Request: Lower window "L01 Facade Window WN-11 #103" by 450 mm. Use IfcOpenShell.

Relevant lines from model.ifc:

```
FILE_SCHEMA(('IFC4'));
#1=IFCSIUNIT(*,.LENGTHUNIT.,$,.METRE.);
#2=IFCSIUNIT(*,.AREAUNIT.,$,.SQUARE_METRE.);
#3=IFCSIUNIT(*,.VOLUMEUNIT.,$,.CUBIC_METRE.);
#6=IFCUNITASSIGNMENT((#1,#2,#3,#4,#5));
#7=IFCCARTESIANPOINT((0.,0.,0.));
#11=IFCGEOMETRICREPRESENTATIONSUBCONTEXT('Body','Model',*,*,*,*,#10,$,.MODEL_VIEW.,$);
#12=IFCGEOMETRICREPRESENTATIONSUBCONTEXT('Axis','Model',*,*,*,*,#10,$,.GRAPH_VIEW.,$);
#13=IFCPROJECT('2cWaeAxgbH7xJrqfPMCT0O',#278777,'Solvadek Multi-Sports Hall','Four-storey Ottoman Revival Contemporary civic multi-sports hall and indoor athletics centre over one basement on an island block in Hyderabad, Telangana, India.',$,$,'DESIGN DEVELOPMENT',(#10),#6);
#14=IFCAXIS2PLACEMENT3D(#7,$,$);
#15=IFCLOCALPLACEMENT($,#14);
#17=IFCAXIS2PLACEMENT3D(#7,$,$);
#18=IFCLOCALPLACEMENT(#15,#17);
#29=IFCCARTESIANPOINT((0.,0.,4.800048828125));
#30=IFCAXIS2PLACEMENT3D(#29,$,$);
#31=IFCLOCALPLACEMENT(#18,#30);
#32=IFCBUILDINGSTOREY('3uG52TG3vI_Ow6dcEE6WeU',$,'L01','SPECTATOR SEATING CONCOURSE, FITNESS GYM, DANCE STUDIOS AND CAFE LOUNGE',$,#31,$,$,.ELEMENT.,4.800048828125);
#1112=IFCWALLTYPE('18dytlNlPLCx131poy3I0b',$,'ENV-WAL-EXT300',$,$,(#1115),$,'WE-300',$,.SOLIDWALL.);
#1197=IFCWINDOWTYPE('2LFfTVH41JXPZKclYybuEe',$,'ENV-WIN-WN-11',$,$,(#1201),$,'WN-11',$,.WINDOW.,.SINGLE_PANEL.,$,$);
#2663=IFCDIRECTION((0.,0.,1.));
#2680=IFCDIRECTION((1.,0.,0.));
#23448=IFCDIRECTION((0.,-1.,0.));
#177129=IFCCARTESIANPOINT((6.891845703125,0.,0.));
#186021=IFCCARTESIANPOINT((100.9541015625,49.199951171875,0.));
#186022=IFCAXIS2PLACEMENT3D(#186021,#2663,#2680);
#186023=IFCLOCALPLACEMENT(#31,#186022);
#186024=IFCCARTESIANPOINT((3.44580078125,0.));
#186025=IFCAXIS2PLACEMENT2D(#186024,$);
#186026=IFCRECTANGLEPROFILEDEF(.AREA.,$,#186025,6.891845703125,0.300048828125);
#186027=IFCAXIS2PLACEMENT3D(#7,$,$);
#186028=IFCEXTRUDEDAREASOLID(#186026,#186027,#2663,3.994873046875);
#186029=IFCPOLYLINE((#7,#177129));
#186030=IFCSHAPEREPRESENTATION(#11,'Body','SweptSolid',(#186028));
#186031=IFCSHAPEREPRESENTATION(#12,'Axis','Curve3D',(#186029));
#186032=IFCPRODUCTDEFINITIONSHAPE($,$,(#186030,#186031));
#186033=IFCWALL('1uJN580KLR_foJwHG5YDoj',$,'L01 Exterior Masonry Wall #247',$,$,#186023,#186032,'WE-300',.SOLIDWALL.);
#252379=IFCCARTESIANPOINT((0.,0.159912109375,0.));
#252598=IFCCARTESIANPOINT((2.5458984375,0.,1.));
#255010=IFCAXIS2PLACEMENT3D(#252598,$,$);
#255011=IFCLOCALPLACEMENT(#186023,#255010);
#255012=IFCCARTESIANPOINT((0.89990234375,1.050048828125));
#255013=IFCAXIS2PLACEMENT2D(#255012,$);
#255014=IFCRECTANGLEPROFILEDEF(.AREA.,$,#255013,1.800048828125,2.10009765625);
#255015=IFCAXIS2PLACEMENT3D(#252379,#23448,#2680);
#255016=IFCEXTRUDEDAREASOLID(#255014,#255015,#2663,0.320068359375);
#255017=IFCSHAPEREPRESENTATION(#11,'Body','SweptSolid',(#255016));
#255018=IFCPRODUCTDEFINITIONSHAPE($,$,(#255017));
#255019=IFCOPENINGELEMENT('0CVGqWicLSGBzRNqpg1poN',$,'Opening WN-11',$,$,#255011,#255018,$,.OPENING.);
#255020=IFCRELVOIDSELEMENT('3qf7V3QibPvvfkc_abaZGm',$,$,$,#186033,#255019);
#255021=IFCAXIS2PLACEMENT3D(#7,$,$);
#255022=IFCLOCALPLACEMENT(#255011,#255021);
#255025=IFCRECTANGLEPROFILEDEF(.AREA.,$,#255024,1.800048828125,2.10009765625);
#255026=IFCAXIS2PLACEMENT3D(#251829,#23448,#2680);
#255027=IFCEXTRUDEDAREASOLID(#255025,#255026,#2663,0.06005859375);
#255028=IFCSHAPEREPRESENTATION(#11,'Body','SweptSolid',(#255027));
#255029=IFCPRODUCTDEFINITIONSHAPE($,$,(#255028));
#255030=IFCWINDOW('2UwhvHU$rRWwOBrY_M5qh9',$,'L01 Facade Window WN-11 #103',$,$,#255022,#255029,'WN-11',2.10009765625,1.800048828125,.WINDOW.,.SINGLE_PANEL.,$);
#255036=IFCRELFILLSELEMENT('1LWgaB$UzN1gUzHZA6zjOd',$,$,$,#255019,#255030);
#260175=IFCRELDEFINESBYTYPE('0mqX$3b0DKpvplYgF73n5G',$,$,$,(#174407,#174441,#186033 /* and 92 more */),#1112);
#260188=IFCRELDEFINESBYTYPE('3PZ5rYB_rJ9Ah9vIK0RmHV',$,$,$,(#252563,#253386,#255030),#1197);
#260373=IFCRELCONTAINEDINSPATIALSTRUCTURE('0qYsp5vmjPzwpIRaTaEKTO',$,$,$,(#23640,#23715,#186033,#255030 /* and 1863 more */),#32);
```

```python
import numpy as np
import ifcopenshell
import ifcopenshell.api.geometry
import ifcopenshell.util.placement
import ifcopenshell.util.unit

model = ifcopenshell.open("model.ifc")
unit_scale = ifcopenshell.util.unit.calculate_unit_scale(model)

window = model.by_guid("2UwhvHU$rRWwOBrY_M5qh9")
opening = window.FillsVoids[0].RelatingOpeningElement
dz = -0.45 / unit_scale

shift = np.array([0.0, 0.0, dz])
# The window is placed relative to its opening, so it follows when the opening moves.
matrix = ifcopenshell.util.placement.get_local_placement(opening.ObjectPlacement)
matrix[:3, 3] += shift
ifcopenshell.api.geometry.edit_object_placement(
    model, product=opening, matrix=matrix, is_si=False, should_transform_children=True
)

print(f"moved by {dz * unit_scale:+.3f} m")

model.write("model_rev.ifc")
```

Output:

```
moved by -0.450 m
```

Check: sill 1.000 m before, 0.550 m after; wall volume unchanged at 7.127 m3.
